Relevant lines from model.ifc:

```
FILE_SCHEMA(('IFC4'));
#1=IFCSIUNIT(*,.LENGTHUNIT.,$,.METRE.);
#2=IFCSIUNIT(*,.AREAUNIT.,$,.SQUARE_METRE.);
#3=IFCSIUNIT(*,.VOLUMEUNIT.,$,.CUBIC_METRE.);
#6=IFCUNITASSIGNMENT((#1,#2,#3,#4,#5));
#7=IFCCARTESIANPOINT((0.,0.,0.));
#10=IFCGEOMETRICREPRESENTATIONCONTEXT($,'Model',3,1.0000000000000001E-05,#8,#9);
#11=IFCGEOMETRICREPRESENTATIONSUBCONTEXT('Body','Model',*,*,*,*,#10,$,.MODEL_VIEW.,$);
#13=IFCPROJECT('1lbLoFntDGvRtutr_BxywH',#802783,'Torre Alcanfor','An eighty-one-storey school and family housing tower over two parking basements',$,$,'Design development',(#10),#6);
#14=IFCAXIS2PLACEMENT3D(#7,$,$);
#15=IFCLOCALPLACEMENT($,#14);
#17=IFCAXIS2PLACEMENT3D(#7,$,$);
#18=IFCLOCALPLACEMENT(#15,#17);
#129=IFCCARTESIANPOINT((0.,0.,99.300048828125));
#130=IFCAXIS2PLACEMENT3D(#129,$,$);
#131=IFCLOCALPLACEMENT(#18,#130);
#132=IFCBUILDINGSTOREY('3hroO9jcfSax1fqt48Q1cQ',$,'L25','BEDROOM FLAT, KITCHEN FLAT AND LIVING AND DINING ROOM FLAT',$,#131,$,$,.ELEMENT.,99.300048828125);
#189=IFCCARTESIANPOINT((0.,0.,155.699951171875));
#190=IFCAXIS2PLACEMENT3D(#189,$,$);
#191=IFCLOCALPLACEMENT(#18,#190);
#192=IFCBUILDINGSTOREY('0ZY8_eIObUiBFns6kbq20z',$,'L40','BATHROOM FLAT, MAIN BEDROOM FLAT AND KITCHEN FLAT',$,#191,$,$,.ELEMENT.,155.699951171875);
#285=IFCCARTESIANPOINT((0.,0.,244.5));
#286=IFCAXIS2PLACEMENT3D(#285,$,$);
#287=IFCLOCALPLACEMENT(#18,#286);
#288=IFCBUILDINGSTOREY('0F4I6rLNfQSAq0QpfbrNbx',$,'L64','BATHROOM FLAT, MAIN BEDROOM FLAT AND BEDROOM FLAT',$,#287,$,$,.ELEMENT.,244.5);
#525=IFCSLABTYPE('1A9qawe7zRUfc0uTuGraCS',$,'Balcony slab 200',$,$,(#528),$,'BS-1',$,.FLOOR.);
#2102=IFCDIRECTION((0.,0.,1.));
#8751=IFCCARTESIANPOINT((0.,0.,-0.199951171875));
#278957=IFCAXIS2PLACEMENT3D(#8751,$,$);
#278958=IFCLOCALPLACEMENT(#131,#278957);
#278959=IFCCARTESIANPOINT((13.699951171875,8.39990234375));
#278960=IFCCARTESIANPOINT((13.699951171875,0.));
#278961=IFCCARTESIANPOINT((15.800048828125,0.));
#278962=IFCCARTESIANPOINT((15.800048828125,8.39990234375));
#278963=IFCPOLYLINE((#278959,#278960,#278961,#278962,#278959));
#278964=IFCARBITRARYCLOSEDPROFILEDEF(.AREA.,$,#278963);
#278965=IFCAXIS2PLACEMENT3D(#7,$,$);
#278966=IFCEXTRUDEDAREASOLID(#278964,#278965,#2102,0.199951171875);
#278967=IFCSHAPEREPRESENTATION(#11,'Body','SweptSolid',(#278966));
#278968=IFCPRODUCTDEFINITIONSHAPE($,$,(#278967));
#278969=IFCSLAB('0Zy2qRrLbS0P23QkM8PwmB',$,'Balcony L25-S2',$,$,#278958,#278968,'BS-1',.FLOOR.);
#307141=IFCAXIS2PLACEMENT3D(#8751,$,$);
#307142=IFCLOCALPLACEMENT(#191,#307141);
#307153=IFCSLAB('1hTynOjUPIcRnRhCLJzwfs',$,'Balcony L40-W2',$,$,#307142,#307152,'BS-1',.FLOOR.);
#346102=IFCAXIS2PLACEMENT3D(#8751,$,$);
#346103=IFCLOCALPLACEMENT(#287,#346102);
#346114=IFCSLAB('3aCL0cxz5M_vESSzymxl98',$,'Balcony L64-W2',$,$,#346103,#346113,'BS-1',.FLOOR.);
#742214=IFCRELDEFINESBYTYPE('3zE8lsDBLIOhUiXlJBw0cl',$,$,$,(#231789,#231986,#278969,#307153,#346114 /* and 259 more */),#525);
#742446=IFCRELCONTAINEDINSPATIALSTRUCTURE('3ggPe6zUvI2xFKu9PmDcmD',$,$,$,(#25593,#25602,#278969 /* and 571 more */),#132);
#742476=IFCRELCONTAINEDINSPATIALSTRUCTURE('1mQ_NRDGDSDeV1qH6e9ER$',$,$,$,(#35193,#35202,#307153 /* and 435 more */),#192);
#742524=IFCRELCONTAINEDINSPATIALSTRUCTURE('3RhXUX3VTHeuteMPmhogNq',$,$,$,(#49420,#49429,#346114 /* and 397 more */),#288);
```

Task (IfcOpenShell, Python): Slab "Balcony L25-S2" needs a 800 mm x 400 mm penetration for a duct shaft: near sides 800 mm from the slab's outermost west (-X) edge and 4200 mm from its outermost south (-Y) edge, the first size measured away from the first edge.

```python
import numpy as np
import ifcopenshell
import ifcopenshell.api.feature
import ifcopenshell.api.geometry
import ifcopenshell.api.root
import ifcopenshell.geom
import ifcopenshell.util.placement
import ifcopenshell.util.representation
import ifcopenshell.util.shape
import ifcopenshell.util.unit

model = ifcopenshell.open("model.ifc")
unit_scale = ifcopenshell.util.unit.calculate_unit_scale(model)
settings = ifcopenshell.geom.settings()


def volume(element):
    """Net volume in cubic metres, openings subtracted."""
    shape = ifcopenshell.geom.create_shape(settings, element)
    return ifcopenshell.util.shape.get_volume(shape.geometry)


slab = model.by_id(278969)
before = volume(slab)

# Extent in the slab's own axes, in metres. The edges named are its -X and -Y sides.
slab_shape = ifcopenshell.geom.create_shape(settings, slab)
vertices = ifcopenshell.util.shape.get_vertices(slab_shape.geometry)
x_min, y_min, bottom = vertices.min(axis=0)
top = vertices[:, 2].max()

opening = ifcopenshell.api.root.create_entity(model, ifc_class="IfcOpeningElement", name="Duct shaft opening", predefined_type="OPENING")
context = ifcopenshell.util.representation.get_context(model, "Model", "Body", "MODEL_VIEW")
width, depth = 0.8, 0.4
outline = [(0.0, 0.0), (width, 0.0), (width, depth), (0.0, depth), (0.0, 0.0)]
# Overshoot both faces by 50 mm so the cut is clean.
shape = ifcopenshell.api.geometry.add_slab_representation(
    model, context=context, depth=top - bottom + 0.1, polyline=outline
)
ifcopenshell.api.geometry.assign_representation(model, product=opening, representation=shape)

matrix = ifcopenshell.util.placement.get_local_placement(slab.ObjectPlacement)
matrix[:, 3] = matrix @ np.append(np.array([x_min + 0.8, y_min + 4.2, bottom - 0.05]) / unit_scale, 1.0)
ifcopenshell.api.geometry.edit_object_placement(model, product=opening, matrix=matrix, is_si=False)
ifcopenshell.api.feature.add_feature(model, feature=opening, element=slab)

after = volume(slab)

print(f"slab volume {before:.3f} -> {after:.3f} m3")

model.write("model_edited.ifc")
```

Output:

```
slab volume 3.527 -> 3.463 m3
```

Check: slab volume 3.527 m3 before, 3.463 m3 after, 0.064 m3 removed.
